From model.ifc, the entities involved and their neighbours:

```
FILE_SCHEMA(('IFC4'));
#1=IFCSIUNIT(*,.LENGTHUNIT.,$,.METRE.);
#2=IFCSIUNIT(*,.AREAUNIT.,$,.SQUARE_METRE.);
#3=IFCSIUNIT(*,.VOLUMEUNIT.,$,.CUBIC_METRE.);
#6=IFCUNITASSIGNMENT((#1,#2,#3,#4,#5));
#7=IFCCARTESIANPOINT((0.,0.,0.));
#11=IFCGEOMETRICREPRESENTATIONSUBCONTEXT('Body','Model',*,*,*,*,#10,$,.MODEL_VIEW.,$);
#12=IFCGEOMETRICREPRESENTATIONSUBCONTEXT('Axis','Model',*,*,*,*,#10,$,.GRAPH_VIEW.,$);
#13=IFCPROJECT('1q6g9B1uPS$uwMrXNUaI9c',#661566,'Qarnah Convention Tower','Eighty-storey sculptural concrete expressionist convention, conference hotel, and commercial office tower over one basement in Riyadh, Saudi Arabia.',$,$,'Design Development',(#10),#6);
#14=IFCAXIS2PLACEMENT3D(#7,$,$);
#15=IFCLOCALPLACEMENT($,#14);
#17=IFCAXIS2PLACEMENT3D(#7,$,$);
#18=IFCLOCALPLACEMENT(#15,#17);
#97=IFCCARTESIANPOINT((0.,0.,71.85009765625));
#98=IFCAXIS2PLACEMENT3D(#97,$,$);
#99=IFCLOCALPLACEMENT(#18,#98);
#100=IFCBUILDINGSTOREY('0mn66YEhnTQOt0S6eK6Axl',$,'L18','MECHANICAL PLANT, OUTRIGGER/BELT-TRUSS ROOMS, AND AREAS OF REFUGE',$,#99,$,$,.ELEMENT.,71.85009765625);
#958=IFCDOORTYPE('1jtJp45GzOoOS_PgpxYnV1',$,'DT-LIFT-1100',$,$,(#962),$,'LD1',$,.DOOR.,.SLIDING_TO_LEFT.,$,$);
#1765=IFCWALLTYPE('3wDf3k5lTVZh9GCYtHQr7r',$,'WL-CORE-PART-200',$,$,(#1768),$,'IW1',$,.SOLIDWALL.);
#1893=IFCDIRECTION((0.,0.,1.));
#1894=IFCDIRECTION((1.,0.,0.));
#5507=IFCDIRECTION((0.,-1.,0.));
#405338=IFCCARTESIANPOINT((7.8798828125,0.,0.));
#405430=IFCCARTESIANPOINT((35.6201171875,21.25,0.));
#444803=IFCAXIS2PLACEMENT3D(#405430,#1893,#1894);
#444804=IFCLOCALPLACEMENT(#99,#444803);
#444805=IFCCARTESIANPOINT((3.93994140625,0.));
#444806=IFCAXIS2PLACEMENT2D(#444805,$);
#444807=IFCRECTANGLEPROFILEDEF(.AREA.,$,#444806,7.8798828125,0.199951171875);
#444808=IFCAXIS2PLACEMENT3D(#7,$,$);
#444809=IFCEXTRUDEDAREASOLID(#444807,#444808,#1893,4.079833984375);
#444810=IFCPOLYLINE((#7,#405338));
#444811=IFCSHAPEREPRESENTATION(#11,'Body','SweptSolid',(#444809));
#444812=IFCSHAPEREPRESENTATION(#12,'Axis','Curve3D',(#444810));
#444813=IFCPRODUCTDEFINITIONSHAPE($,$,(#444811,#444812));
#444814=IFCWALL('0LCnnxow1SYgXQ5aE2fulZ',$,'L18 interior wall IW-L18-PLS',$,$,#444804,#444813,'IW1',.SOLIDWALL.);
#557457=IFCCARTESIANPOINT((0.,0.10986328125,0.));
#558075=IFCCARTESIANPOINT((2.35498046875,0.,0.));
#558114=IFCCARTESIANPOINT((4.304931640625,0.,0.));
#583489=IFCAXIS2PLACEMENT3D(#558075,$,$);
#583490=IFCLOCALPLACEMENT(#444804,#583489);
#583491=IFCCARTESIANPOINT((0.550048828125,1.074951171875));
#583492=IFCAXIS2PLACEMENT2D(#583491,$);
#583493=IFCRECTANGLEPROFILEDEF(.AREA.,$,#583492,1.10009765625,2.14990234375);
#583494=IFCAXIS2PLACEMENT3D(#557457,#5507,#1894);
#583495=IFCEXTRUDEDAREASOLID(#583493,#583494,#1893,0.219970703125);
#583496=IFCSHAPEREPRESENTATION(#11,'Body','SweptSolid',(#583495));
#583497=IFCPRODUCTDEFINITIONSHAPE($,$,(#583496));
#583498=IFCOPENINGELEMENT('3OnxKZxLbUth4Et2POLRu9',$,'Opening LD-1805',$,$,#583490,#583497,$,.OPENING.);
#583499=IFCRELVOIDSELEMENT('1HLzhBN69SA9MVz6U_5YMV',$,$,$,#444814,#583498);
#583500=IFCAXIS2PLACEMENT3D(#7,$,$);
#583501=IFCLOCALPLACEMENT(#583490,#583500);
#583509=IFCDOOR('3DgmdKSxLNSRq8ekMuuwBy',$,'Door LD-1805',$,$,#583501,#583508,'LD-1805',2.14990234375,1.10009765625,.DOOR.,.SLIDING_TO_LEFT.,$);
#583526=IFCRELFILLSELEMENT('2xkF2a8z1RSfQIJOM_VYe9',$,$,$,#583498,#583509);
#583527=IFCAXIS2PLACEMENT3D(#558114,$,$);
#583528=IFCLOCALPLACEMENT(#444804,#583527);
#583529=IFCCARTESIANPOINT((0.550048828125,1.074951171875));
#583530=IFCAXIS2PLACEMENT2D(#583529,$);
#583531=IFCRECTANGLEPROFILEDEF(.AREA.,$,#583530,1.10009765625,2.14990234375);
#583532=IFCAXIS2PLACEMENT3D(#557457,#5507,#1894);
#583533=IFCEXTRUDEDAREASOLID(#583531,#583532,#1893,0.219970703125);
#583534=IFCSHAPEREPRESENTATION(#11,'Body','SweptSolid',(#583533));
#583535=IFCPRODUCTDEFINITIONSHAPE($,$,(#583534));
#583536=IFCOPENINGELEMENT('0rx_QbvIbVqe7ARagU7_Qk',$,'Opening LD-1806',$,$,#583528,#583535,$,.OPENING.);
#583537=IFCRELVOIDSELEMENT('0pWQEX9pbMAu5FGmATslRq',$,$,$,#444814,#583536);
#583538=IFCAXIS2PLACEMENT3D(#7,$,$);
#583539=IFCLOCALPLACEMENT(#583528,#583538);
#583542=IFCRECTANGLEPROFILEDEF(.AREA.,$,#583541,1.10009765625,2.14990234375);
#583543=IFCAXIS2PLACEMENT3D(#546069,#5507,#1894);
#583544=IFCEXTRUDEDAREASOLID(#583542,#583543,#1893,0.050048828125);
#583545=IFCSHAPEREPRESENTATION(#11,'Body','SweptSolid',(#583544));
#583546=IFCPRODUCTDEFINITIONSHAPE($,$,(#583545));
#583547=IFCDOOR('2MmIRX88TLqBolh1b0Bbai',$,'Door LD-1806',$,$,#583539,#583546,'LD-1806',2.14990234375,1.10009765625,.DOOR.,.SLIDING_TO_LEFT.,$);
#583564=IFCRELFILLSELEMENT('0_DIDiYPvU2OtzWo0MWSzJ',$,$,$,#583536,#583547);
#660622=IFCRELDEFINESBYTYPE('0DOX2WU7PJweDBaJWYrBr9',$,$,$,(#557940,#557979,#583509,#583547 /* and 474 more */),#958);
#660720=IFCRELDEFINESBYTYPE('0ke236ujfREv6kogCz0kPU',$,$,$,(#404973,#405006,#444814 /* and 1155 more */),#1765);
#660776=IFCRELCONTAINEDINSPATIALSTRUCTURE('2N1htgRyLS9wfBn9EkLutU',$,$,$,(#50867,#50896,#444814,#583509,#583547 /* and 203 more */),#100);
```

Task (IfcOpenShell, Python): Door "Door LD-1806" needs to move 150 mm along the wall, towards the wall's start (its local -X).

```python
import ifcopenshell
import ifcopenshell.api.geometry
import ifcopenshell.util.placement

model = ifcopenshell.open("model.ifc")

door = model.by_guid("2MmIRX88TLqBolh1b0Bbai")
opening = door.FillsVoids[0].RelatingOpeningElement
wall = opening.VoidsElements[0].RelatingBuildingElement

wall_matrix = ifcopenshell.util.placement.get_local_placement(wall.ObjectPlacement)
shift = wall_matrix[:3, 0] * -0.15
before = ifcopenshell.util.placement.get_local_placement(door.ObjectPlacement)[:3, 3].copy()

# The door is placed relative to its opening, so it follows when the opening moves.
matrix = ifcopenshell.util.placement.get_local_placement(opening.ObjectPlacement)
matrix[:3, 3] += shift
ifcopenshell.api.geometry.edit_object_placement(
    model, product=opening, matrix=matrix, is_si=False, should_transform_children=True
)

after = ifcopenshell.util.placement.get_local_placement(door.ObjectPlacement)[:3, 3]
print("door moved by", (after - before).round(3) + 0.0)

model.write("model_rev.ifc")
```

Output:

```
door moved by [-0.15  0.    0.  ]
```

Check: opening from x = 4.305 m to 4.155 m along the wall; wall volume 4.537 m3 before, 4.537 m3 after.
